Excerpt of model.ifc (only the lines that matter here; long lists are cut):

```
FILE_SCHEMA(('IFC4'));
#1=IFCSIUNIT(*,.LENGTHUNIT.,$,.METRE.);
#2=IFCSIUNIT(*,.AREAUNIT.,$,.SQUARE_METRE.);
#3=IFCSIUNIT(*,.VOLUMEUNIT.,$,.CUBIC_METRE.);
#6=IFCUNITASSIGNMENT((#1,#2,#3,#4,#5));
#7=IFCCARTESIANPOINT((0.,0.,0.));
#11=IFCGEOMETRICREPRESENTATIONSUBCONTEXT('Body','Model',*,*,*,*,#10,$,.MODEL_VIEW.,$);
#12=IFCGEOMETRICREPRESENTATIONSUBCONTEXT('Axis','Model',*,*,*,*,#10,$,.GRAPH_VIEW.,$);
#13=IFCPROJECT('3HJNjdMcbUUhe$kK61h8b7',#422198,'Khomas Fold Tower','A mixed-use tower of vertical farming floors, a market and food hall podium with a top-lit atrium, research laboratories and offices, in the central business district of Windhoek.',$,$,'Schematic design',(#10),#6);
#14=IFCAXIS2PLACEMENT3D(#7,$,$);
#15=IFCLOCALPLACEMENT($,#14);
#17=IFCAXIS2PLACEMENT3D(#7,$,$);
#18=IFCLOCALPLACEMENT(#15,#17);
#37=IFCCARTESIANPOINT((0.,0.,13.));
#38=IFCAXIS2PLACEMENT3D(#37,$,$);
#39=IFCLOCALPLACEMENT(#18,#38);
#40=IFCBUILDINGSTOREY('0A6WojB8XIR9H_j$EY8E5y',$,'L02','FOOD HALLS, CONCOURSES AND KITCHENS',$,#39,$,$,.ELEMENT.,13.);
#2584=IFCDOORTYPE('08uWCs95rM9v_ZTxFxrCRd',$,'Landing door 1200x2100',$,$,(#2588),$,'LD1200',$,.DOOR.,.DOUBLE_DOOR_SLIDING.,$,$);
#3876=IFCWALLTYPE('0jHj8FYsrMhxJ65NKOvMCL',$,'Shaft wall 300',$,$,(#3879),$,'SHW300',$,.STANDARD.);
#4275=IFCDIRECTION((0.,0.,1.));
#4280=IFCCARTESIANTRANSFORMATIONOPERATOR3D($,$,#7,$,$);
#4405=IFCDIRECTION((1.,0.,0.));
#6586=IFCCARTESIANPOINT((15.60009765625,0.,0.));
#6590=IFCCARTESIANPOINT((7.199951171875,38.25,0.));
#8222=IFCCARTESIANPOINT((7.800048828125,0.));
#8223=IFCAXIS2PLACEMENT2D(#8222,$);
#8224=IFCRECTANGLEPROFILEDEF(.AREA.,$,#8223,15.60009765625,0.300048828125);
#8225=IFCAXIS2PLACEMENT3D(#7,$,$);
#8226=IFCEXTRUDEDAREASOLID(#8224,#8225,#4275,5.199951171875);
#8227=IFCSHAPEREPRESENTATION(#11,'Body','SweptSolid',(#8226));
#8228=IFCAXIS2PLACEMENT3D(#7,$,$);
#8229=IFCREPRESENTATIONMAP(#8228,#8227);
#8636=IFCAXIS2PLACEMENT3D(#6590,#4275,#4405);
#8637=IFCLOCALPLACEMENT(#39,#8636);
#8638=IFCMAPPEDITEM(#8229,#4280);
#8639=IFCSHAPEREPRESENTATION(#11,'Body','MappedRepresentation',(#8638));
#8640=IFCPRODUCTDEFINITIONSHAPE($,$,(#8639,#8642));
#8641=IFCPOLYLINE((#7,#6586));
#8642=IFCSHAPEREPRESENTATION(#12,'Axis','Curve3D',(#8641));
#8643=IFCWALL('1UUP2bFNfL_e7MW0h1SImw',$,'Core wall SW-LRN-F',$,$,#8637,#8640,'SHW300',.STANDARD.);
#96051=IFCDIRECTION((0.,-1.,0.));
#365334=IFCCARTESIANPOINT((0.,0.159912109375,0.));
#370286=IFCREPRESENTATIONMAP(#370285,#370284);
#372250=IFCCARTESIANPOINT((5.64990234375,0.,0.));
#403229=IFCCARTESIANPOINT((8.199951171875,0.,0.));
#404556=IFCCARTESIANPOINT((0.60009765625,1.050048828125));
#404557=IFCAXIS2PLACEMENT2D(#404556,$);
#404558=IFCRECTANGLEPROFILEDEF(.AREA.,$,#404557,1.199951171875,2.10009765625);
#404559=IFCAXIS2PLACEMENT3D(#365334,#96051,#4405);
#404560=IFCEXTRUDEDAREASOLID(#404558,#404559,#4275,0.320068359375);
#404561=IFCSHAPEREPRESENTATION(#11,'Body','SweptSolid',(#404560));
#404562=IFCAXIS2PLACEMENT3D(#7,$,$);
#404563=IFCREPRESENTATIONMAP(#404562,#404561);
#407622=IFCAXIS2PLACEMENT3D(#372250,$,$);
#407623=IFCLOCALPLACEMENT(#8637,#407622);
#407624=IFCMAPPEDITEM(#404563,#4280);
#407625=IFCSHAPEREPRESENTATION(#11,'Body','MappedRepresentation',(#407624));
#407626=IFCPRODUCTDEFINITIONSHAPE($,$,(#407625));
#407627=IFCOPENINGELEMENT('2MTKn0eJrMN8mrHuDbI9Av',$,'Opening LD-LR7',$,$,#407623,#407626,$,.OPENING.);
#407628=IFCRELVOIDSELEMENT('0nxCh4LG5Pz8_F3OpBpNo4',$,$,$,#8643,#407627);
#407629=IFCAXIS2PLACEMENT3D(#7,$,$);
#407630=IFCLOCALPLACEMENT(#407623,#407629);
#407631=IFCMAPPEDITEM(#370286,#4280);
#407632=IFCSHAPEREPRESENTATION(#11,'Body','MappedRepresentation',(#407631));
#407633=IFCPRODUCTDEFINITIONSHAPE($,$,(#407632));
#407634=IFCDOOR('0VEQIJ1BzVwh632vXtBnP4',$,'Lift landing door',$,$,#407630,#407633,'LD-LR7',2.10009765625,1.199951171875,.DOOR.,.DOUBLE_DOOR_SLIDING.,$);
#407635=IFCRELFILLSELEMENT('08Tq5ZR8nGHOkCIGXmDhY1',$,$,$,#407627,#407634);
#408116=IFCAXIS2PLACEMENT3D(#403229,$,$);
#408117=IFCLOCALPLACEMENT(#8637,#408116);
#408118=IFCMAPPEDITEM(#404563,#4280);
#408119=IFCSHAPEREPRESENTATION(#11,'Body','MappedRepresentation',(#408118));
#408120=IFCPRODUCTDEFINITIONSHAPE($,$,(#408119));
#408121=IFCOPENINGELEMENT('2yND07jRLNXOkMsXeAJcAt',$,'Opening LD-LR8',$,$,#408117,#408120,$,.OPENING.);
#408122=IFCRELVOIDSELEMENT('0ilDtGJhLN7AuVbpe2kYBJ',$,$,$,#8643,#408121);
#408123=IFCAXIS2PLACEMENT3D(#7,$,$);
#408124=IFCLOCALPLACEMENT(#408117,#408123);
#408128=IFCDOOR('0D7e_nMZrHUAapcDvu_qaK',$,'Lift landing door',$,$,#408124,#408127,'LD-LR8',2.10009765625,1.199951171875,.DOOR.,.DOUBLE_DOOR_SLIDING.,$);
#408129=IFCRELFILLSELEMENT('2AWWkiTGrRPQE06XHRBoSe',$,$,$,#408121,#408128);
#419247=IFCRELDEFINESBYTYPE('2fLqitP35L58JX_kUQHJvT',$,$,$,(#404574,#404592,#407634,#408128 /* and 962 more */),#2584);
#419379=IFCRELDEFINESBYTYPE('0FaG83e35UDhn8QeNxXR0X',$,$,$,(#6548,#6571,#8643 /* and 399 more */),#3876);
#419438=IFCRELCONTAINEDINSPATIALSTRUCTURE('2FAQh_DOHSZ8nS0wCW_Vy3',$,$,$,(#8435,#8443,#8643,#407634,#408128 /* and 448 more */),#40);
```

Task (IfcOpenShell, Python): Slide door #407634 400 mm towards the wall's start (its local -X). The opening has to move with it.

```python
import ifcopenshell
import ifcopenshell.api.geometry
import ifcopenshell.util.placement
import ifcopenshell.util.unit

model = ifcopenshell.open("model.ifc")
unit_scale = ifcopenshell.util.unit.calculate_unit_scale(model)

door = model.by_guid("0VEQIJ1BzVwh632vXtBnP4")
opening = door.FillsVoids[0].RelatingOpeningElement
wall = opening.VoidsElements[0].RelatingBuildingElement

wall_matrix = ifcopenshell.util.placement.get_local_placement(wall.ObjectPlacement)
shift = wall_matrix[:3, 0] * -0.4 / unit_scale
before = ifcopenshell.util.placement.get_local_placement(door.ObjectPlacement)[:3, 3].copy()

# The door is placed relative to its opening, so it follows when the opening moves.
matrix = ifcopenshell.util.placement.get_local_placement(opening.ObjectPlacement)
matrix[:3, 3] += shift
ifcopenshell.api.geometry.edit_object_placement(
    model, product=opening, matrix=matrix, is_si=False, should_transform_children=True
)

after = ifcopenshell.util.placement.get_local_placement(door.ObjectPlacement)[:3, 3]
print("door moved by", (after - before).round(3) + 0.0)

model.write("model_v2.ifc")
```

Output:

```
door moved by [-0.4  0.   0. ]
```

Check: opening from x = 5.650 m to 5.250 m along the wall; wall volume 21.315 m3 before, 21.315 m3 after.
